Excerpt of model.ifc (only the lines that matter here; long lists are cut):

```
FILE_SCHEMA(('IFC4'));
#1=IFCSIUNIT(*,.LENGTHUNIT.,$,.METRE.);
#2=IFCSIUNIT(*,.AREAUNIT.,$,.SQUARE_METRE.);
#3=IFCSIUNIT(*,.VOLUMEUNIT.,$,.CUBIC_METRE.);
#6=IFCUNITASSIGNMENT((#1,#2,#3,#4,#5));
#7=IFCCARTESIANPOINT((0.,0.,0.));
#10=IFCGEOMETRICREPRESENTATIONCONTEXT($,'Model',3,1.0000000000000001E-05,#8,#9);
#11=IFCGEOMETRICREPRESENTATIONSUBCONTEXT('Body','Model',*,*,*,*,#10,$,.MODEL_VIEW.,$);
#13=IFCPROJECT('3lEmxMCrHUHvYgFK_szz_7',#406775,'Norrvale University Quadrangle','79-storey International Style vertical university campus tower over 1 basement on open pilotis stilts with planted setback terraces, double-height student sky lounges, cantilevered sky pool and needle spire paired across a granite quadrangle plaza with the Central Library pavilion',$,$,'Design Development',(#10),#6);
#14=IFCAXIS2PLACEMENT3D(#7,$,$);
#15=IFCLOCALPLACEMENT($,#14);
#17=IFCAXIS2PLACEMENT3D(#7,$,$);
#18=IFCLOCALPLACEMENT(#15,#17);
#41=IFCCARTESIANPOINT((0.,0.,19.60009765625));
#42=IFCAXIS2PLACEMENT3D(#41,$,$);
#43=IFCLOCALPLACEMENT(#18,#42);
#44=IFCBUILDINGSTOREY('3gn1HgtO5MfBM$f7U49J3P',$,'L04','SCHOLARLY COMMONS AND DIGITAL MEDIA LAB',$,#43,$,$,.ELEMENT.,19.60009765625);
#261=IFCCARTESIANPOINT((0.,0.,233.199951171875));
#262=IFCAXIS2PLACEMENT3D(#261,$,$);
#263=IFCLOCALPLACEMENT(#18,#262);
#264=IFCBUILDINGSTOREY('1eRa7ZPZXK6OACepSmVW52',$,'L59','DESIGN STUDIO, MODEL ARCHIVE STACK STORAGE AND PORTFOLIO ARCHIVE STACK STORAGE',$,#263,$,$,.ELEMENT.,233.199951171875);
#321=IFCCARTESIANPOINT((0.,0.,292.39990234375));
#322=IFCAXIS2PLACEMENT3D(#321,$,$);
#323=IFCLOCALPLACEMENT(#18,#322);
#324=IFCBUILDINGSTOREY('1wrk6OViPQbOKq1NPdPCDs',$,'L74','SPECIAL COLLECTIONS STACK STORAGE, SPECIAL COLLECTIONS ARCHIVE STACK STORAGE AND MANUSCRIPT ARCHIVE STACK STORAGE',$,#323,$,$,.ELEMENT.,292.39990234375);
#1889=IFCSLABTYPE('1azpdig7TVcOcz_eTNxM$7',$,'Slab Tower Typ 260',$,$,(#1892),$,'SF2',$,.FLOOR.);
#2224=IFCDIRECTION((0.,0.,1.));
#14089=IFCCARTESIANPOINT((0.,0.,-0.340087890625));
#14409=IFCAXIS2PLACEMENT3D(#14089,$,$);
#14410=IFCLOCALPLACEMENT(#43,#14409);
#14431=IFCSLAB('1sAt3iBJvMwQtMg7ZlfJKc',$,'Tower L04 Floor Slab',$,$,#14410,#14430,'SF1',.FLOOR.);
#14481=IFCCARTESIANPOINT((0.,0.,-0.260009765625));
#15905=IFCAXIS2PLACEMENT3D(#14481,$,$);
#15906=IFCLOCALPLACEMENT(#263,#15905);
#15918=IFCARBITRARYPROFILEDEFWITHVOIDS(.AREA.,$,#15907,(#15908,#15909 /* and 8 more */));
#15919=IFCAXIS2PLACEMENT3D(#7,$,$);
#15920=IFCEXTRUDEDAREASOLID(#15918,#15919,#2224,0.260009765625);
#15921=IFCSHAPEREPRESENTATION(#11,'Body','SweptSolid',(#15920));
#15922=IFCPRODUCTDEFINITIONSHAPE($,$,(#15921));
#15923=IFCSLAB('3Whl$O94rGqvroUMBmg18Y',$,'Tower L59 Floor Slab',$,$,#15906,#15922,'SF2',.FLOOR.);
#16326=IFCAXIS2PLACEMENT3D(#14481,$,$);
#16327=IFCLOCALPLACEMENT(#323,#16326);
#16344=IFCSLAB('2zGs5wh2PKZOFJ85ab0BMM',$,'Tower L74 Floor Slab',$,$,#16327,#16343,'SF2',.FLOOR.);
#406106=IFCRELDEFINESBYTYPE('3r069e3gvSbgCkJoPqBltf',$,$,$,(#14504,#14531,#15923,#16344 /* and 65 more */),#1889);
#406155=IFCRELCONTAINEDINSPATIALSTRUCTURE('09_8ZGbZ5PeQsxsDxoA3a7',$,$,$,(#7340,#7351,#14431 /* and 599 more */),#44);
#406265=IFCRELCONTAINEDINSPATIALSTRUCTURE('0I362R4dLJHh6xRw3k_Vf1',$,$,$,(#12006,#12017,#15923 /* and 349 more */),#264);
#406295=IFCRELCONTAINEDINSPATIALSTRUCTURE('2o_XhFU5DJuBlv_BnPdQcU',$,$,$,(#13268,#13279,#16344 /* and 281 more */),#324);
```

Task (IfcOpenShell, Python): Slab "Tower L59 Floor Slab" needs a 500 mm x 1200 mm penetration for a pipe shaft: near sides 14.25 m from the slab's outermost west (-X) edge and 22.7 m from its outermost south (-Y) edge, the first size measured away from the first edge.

```python
import numpy as np
import ifcopenshell
import ifcopenshell.api.feature
import ifcopenshell.api.geometry
import ifcopenshell.api.root
import ifcopenshell.geom
import ifcopenshell.util.placement
import ifcopenshell.util.representation
import ifcopenshell.util.shape
import ifcopenshell.util.unit

model = ifcopenshell.open("model.ifc")
unit_scale = ifcopenshell.util.unit.calculate_unit_scale(model)
settings = ifcopenshell.geom.settings()


def volume(element):
    """Net volume in cubic metres, openings subtracted."""
    shape = ifcopenshell.geom.create_shape(settings, element)
    return ifcopenshell.util.shape.get_volume(shape.geometry)


slab = model.by_guid("3Whl$O94rGqvroUMBmg18Y")
before = volume(slab)

# Extent in the slab's own axes, in metres. The edges named are its -X and -Y sides.
slab_shape = ifcopenshell.geom.create_shape(settings, slab)
vertices = ifcopenshell.util.shape.get_vertices(slab_shape.geometry)
x_min, y_min, bottom = vertices.min(axis=0)
top = vertices[:, 2].max()

opening = ifcopenshell.api.root.create_entity(model, ifc_class="IfcOpeningElement", name="Pipe shaft opening", predefined_type="OPENING")
context = ifcopenshell.util.representation.get_context(model, "Model", "Body", "MODEL_VIEW")
width, depth = 0.5, 1.2
outline = [(0.0, 0.0), (width, 0.0), (width, depth), (0.0, depth), (0.0, 0.0)]
# Overshoot both faces by 50 mm so the cut is clean.
shape = ifcopenshell.api.geometry.add_slab_representation(
    model, context=context, depth=top - bottom + 0.1, polyline=outline
)
ifcopenshell.api.geometry.assign_representation(model, product=opening, representation=shape)

matrix = ifcopenshell.util.placement.get_local_placement(slab.ObjectPlacement)
matrix[:, 3] = matrix @ np.append(np.array([x_min + 14.25, y_min + 22.7, bottom - 0.05]) / unit_scale, 1.0)
ifcopenshell.api.geometry.edit_object_placement(model, product=opening, matrix=matrix, is_si=False)
ifcopenshell.api.feature.add_feature(model, feature=opening, element=slab)

after = volume(slab)

print(f"slab volume {before:.3f} -> {after:.3f} m3")

model.write("model-out.ifc")
```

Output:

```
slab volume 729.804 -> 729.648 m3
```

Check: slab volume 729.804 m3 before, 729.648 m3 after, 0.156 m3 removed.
